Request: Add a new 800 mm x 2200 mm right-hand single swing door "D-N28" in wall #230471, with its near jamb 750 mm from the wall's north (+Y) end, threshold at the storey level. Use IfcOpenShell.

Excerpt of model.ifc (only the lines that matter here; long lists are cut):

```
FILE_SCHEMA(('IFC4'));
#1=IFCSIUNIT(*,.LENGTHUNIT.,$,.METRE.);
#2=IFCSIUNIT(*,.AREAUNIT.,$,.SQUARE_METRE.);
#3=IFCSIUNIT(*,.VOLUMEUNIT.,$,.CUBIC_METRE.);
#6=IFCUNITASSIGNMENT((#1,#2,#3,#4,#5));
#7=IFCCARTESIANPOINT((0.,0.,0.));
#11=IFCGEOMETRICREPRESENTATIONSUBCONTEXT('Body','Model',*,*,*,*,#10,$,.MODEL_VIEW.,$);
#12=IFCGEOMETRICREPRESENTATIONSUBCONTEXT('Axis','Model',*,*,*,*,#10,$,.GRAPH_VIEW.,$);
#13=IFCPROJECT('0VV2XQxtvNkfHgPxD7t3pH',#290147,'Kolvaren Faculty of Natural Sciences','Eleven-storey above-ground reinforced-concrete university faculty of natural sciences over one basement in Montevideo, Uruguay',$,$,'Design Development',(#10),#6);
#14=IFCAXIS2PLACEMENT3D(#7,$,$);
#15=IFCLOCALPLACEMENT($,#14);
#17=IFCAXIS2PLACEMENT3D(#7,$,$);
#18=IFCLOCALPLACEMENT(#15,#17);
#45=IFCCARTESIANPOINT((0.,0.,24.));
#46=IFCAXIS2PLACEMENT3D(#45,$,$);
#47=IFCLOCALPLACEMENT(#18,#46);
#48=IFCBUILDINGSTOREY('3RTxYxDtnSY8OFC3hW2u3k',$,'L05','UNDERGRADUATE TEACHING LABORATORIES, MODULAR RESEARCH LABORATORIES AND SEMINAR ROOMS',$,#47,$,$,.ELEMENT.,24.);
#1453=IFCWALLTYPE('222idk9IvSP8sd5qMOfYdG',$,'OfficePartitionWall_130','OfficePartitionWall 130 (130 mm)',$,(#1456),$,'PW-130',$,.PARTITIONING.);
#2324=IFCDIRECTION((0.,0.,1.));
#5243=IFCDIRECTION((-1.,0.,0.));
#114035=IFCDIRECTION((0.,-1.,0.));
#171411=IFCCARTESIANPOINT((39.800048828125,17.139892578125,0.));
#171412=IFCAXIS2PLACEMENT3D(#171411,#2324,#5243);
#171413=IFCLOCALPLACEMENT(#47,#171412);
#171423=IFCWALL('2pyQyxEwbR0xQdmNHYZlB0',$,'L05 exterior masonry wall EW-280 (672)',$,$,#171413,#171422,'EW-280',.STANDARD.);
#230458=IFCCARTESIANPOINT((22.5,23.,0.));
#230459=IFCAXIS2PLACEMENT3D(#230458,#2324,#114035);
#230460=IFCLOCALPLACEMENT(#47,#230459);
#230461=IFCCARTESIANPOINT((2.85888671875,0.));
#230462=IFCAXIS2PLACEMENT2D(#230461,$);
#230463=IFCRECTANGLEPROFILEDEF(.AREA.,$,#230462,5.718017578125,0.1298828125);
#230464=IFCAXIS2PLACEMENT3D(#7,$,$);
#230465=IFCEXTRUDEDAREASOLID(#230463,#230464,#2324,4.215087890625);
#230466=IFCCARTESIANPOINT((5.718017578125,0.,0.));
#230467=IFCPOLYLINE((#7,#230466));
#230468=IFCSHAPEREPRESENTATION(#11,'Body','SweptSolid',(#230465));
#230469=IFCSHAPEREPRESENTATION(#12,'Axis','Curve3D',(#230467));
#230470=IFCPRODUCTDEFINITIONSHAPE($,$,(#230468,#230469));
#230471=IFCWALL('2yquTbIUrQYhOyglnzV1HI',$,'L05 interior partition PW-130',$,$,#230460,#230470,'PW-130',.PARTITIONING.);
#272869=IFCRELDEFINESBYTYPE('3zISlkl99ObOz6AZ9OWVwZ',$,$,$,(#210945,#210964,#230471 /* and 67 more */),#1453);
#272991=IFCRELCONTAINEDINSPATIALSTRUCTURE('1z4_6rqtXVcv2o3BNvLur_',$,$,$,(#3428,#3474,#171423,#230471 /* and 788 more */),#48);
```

```python
import numpy as np
import ifcopenshell
import ifcopenshell.api.feature
import ifcopenshell.api.geometry
import ifcopenshell.api.root
import ifcopenshell.api.spatial
import ifcopenshell.geom
import ifcopenshell.util.element
import ifcopenshell.util.placement
import ifcopenshell.util.representation
import ifcopenshell.util.shape
import ifcopenshell.util.unit

model = ifcopenshell.open("model.ifc")
unit_scale = ifcopenshell.util.unit.calculate_unit_scale(model)
settings = ifcopenshell.geom.settings()


def volume(element):
    """Net volume in cubic metres, openings subtracted."""
    shape = ifcopenshell.geom.create_shape(settings, element)
    return ifcopenshell.util.shape.get_volume(shape.geometry)


wall = model.by_guid("2yquTbIUrQYhOyglnzV1HI")
storey = ifcopenshell.util.element.get_container(wall, ifc_class="IfcBuildingStorey")
context = ifcopenshell.util.representation.get_context(model, "Model", "Body", "MODEL_VIEW")
before = volume(wall)

width, height, from_end, sill = 0.8, 2.2, 0.75, 0.0  # metres

# The wall runs along its own X axis, and the end named is its -X end.
wall_shape = ifcopenshell.geom.create_shape(settings, wall)
x, y, z = ifcopenshell.util.shape.get_vertices(wall_shape.geometry).T
start = x.min() + from_end
face, thickness = float(y.min()), float(y.max() - y.min())
wall_matrix = ifcopenshell.util.placement.get_local_placement(wall.ObjectPlacement)
level = ifcopenshell.util.placement.get_local_placement(storey.ObjectPlacement)[2, 3]


def in_wall(x, y):
    """Placement at x, y metres in the wall's axes, at sill height."""
    matrix = wall_matrix.copy()
    matrix[:, 3] = wall_matrix @ np.array([x / unit_scale, y / unit_scale, 0.0, 1.0])
    matrix[2, 3] = level + sill / unit_scale
    return matrix


# Opening: a box that overshoots both wall faces by 50 mm.
opening = ifcopenshell.api.root.create_entity(model, ifc_class="IfcOpeningElement", predefined_type="OPENING")
box = ifcopenshell.api.geometry.add_wall_representation(
    model, context=context, length=width, height=height, thickness=thickness + 0.1
)
ifcopenshell.api.geometry.assign_representation(model, product=opening, representation=box)
ifcopenshell.api.geometry.edit_object_placement(model, product=opening, matrix=in_wall(start, face - 0.05), is_si=False)
ifcopenshell.api.feature.add_feature(model, feature=opening, element=wall)

door = ifcopenshell.api.root.create_entity(model, ifc_class="IfcDoor", name="D-N28", predefined_type="DOOR")
door.OverallWidth, door.OverallHeight = width / unit_scale, height / unit_scale
door.OperationType = "SINGLE_SWING_RIGHT"
body = ifcopenshell.api.geometry.add_door_representation(
    model,
    context=context,
    overall_width=door.OverallWidth,
    overall_height=door.OverallHeight,
    operation_type="SINGLE_SWING_RIGHT",
    lining_properties={"LiningDepth": thickness / unit_scale, "ThresholdDepth": thickness / unit_scale},
)
ifcopenshell.api.geometry.assign_representation(model, product=door, representation=body)
ifcopenshell.api.spatial.assign_container(model, products=[door], relating_structure=storey)
ifcopenshell.api.feature.add_filling(model, opening=opening, element=door)

# The lining spans the wall, so the door starts at the wall face.
ifcopenshell.api.geometry.edit_object_placement(model, product=door, matrix=in_wall(start, face), is_si=False)

after = volume(wall)

print(f"wall volume {before:.3f} -> {after:.3f} m3")

model.write("model_v2.ifc")
```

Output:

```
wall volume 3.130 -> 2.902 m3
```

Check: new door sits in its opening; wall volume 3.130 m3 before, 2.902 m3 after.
